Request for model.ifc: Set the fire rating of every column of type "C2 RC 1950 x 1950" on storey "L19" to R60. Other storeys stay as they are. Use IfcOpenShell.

First a look at what the model holds.

```python
import ifcopenshell
import ifcopenshell.util.element

model = ifcopenshell.open("model.ifc")
print(model.schema)
storey = next(s for s in model.by_type("IfcBuildingStorey") if s.Name == "L19")
columns = [e for e in ifcopenshell.util.element.get_decomposition(storey) if e.is_a("IfcColumn")]
seen = {}
for e in columns:
    element_type = ifcopenshell.util.element.get_type(e)
    key = (element_type.Name if element_type != e and element_type else None, ifcopenshell.util.element.get_pset(e, "Pset_ColumnCommon", "FireRating"))
    seen[key] = seen.get(key, 0) + 1
for (name, value), count in sorted(seen.items(), key=str):
    print(count, "x", name, "|", value)
```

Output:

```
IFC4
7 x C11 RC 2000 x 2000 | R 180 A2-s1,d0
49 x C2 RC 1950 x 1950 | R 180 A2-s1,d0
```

```python
import ifcopenshell
import ifcopenshell.api.pset
import ifcopenshell.util.element

model = ifcopenshell.open("model.ifc")

storey = next(s for s in model.by_type("IfcBuildingStorey") if s.Name == "L19")
columns = [e for e in ifcopenshell.util.element.get_decomposition(storey) if e.is_a("IfcColumn")]

count = 0
for e in columns:
    element_type = ifcopenshell.util.element.get_type(e)
    if element_type in (None, e) or element_type.Name != "C2 RC 1950 x 1950":
        continue
    found = ifcopenshell.util.element.get_pset(e, "Pset_ColumnCommon", should_inherit=False)
    if found:
        pset = model.by_id(found["id"])
        if len(ifcopenshell.util.element.get_elements_by_pset(pset)) > 1:
            pset = ifcopenshell.api.pset.unshare_pset(model, products=[e], pset=pset)[0]
    else:
        pset = ifcopenshell.api.pset.add_pset(model, product=e, name="Pset_ColumnCommon")
    ifcopenshell.api.pset.edit_pset(model, pset=pset, properties={"FireRating": "R60"})
    count += 1

print(count, "columns updated")

model.write("model_v2.ifc")
```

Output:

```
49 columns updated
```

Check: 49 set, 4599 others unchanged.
